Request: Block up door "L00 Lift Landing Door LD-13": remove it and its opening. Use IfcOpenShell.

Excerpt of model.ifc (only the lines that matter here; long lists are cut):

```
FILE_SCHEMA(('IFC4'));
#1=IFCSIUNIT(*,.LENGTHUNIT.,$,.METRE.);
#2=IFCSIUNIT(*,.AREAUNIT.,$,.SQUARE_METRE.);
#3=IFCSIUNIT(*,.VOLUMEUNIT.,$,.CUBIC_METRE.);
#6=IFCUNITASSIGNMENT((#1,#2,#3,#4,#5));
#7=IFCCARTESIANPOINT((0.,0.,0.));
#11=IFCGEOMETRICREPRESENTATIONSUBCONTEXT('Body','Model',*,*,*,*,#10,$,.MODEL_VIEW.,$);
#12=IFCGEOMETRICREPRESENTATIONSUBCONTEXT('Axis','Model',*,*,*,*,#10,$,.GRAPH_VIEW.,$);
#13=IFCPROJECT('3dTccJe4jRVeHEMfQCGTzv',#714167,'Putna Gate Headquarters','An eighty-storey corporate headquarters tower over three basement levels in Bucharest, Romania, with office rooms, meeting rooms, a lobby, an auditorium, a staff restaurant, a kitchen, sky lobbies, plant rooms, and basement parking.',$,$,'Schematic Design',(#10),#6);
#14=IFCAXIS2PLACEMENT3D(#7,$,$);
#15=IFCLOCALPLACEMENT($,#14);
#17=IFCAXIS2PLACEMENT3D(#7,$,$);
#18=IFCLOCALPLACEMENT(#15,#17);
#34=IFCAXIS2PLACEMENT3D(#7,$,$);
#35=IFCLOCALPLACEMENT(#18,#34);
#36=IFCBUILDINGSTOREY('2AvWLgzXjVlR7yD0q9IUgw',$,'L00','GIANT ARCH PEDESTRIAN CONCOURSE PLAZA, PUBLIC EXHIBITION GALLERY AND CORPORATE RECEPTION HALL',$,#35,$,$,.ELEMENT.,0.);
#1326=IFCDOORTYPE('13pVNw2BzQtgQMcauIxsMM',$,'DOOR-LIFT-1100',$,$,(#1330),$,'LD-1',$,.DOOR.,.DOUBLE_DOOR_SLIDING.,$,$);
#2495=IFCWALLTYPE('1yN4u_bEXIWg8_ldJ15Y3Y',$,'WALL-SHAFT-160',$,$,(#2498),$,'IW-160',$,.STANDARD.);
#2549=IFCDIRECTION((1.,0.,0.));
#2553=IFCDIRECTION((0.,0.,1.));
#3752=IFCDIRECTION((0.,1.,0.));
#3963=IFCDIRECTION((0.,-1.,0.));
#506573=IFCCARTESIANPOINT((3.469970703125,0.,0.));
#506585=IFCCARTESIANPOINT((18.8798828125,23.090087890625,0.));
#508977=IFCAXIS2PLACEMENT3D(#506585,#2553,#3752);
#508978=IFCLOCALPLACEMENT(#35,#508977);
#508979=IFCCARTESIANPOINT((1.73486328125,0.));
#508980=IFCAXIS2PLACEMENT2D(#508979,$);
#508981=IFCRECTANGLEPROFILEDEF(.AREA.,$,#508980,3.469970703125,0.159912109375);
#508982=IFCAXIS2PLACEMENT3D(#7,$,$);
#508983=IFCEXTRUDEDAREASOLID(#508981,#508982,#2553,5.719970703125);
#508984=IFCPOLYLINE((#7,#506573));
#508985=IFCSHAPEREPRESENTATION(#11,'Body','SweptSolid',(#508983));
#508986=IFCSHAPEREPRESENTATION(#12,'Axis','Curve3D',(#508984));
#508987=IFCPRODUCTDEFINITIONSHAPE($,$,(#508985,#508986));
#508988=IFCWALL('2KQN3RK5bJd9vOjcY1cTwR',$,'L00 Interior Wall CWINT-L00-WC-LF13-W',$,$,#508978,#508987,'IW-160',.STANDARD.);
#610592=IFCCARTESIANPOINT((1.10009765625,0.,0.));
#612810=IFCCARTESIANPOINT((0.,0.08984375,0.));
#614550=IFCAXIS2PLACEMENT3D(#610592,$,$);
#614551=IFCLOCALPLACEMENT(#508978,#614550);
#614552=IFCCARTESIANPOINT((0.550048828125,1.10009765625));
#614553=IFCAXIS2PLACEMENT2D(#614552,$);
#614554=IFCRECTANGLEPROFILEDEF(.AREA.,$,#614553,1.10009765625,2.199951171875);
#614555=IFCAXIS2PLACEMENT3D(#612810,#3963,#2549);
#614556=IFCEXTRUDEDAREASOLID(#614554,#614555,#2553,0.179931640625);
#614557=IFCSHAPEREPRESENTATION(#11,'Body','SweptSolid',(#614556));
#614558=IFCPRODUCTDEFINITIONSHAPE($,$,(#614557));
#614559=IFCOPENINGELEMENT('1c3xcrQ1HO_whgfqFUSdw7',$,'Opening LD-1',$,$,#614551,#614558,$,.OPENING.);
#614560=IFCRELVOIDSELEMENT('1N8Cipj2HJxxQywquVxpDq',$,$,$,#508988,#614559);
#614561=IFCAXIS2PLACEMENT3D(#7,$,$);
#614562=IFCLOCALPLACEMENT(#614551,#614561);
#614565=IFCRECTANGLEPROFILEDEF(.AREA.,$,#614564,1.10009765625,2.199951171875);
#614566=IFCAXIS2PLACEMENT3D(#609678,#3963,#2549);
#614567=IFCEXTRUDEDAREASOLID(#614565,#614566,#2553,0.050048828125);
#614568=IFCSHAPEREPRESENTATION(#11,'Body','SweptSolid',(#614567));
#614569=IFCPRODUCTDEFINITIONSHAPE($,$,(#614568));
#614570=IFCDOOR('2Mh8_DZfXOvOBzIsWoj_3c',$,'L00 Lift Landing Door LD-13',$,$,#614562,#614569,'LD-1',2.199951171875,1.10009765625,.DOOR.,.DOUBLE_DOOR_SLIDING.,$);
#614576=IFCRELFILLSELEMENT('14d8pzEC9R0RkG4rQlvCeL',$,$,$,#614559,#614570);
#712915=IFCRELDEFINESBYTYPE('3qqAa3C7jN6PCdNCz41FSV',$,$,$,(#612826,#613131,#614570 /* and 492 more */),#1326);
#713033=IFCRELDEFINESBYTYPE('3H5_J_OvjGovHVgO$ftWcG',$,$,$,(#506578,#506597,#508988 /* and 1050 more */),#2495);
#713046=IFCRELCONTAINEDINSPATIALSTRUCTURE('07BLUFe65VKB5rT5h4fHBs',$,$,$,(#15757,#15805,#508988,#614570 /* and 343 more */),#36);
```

```python
import ifcopenshell
import ifcopenshell.api.feature
import ifcopenshell.api.root
import ifcopenshell.geom
import ifcopenshell.util.shape

model = ifcopenshell.open("model.ifc")
settings = ifcopenshell.geom.settings()


def volume(element):
    """Net volume in cubic metres, openings subtracted."""
    shape = ifcopenshell.geom.create_shape(settings, element)
    return ifcopenshell.util.shape.get_volume(shape.geometry)


door = model.by_id(614570)
opening = door.FillsVoids[0].RelatingOpeningElement
wall = opening.VoidsElements[0].RelatingBuildingElement
before = volume(wall)

ifcopenshell.api.root.remove_product(model, product=door)
ifcopenshell.api.feature.remove_feature(model, feature=opening)

after = volume(wall)

print(f"wall volume {before:.3f} -> {after:.3f} m3")

model.write("model_rev.ifc")
```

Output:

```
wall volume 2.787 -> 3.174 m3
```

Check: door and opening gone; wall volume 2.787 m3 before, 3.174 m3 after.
